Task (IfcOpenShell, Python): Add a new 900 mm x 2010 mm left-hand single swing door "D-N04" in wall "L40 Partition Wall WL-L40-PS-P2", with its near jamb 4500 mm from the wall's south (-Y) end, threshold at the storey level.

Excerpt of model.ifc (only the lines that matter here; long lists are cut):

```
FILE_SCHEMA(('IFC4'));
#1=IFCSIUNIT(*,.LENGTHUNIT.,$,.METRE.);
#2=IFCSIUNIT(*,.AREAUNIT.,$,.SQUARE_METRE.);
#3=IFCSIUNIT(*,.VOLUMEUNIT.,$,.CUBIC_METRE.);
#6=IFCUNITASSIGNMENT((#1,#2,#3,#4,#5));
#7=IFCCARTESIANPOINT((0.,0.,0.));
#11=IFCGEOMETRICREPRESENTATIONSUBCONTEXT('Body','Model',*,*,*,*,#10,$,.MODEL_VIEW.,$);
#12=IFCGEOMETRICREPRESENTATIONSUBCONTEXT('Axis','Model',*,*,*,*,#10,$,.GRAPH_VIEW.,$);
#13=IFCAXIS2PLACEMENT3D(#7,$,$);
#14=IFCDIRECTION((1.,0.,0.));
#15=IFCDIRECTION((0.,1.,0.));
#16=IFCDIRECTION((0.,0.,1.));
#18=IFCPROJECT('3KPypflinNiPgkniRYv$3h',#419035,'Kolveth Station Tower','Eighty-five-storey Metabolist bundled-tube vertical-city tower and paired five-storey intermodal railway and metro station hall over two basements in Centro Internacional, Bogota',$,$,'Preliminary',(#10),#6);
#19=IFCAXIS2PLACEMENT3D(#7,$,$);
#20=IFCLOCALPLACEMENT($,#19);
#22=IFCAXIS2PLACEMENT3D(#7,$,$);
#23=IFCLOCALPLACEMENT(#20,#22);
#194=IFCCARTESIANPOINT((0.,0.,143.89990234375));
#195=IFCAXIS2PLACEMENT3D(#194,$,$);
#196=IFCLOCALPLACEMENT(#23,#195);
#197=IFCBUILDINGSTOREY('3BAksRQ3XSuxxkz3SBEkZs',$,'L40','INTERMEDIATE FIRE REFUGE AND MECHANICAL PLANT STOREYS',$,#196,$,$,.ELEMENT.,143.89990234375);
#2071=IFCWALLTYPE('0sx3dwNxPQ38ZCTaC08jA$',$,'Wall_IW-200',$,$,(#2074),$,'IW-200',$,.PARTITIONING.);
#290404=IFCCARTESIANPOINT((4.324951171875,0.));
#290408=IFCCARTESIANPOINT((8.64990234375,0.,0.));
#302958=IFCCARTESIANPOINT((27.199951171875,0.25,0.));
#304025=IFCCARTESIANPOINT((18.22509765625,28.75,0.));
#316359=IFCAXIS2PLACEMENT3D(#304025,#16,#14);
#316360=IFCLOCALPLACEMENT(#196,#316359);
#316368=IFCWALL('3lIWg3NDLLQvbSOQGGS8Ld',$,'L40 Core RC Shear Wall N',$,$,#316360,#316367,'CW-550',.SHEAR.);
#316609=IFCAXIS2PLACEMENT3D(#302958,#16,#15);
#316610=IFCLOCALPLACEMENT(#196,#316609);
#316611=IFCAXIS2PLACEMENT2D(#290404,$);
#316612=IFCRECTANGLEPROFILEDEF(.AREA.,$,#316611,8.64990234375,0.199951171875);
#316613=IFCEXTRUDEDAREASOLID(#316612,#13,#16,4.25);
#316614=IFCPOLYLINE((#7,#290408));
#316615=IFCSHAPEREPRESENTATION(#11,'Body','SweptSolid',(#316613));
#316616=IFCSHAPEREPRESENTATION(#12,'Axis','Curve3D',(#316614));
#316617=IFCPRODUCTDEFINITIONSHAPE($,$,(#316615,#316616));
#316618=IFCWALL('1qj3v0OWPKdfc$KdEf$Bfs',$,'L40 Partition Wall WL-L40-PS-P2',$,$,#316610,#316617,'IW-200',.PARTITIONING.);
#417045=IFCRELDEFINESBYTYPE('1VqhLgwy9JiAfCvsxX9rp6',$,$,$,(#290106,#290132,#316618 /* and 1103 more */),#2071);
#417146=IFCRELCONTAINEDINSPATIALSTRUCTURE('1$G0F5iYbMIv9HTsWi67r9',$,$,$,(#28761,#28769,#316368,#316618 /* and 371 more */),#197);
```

```python
import numpy as np
import ifcopenshell
import ifcopenshell.api.feature
import ifcopenshell.api.geometry
import ifcopenshell.api.root
import ifcopenshell.api.spatial
import ifcopenshell.geom
import ifcopenshell.util.element
import ifcopenshell.util.placement
import ifcopenshell.util.representation
import ifcopenshell.util.shape
import ifcopenshell.util.unit

model = ifcopenshell.open("model.ifc")
unit_scale = ifcopenshell.util.unit.calculate_unit_scale(model)
settings = ifcopenshell.geom.settings()


def volume(element):
    """Net volume in cubic metres, openings subtracted."""
    shape = ifcopenshell.geom.create_shape(settings, element)
    return ifcopenshell.util.shape.get_volume(shape.geometry)


wall = model.by_guid("1qj3v0OWPKdfc$KdEf$Bfs")
storey = ifcopenshell.util.element.get_container(wall, ifc_class="IfcBuildingStorey")
context = ifcopenshell.util.representation.get_context(model, "Model", "Body", "MODEL_VIEW")
before = volume(wall)

width, height, from_end, sill = 0.9, 2.01, 4.5, 0.0  # metres

# The wall runs along its own X axis, and the end named is its -X end.
wall_shape = ifcopenshell.geom.create_shape(settings, wall)
x, y, z = ifcopenshell.util.shape.get_vertices(wall_shape.geometry).T
start = x.min() + from_end
face, thickness = float(y.min()), float(y.max() - y.min())
wall_matrix = ifcopenshell.util.placement.get_local_placement(wall.ObjectPlacement)
level = ifcopenshell.util.placement.get_local_placement(storey.ObjectPlacement)[2, 3]


def in_wall(x, y):
    """Placement at x, y metres in the wall's axes, at sill height."""
    matrix = wall_matrix.copy()
    matrix[:, 3] = wall_matrix @ np.array([x / unit_scale, y / unit_scale, 0.0, 1.0])
    matrix[2, 3] = level + sill / unit_scale
    return matrix


# Opening: a box that overshoots both wall faces by 50 mm.
opening = ifcopenshell.api.root.create_entity(model, ifc_class="IfcOpeningElement", predefined_type="OPENING")
box = ifcopenshell.api.geometry.add_wall_representation(
    model, context=context, length=width, height=height, thickness=thickness + 0.1
)
ifcopenshell.api.geometry.assign_representation(model, product=opening, representation=box)
ifcopenshell.api.geometry.edit_object_placement(model, product=opening, matrix=in_wall(start, face - 0.05), is_si=False)
ifcopenshell.api.feature.add_feature(model, feature=opening, element=wall)

door = ifcopenshell.api.root.create_entity(model, ifc_class="IfcDoor", name="D-N04", predefined_type="DOOR")
door.OverallWidth, door.OverallHeight = width / unit_scale, height / unit_scale
door.OperationType = "SINGLE_SWING_LEFT"
body = ifcopenshell.api.geometry.add_door_representation(
    model,
    context=context,
    overall_width=door.OverallWidth,
    overall_height=door.OverallHeight,
    operation_type="SINGLE_SWING_LEFT",
    lining_properties={"LiningDepth": thickness / unit_scale, "ThresholdDepth": thickness / unit_scale},
)
ifcopenshell.api.geometry.assign_representation(model, product=door, representation=body)
ifcopenshell.api.spatial.assign_container(model, products=[door], relating_structure=storey)
ifcopenshell.api.feature.add_filling(model, opening=opening, element=door)

# The lining spans the wall, so the door starts at the wall face.
ifcopenshell.api.geometry.edit_object_placement(model, product=door, matrix=in_wall(start, face), is_si=False)

after = volume(wall)

print(f"wall volume {before:.3f} -> {after:.3f} m3")

model.write("model_updated.ifc")
```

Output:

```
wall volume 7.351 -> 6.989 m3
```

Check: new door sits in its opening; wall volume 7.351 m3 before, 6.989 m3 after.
